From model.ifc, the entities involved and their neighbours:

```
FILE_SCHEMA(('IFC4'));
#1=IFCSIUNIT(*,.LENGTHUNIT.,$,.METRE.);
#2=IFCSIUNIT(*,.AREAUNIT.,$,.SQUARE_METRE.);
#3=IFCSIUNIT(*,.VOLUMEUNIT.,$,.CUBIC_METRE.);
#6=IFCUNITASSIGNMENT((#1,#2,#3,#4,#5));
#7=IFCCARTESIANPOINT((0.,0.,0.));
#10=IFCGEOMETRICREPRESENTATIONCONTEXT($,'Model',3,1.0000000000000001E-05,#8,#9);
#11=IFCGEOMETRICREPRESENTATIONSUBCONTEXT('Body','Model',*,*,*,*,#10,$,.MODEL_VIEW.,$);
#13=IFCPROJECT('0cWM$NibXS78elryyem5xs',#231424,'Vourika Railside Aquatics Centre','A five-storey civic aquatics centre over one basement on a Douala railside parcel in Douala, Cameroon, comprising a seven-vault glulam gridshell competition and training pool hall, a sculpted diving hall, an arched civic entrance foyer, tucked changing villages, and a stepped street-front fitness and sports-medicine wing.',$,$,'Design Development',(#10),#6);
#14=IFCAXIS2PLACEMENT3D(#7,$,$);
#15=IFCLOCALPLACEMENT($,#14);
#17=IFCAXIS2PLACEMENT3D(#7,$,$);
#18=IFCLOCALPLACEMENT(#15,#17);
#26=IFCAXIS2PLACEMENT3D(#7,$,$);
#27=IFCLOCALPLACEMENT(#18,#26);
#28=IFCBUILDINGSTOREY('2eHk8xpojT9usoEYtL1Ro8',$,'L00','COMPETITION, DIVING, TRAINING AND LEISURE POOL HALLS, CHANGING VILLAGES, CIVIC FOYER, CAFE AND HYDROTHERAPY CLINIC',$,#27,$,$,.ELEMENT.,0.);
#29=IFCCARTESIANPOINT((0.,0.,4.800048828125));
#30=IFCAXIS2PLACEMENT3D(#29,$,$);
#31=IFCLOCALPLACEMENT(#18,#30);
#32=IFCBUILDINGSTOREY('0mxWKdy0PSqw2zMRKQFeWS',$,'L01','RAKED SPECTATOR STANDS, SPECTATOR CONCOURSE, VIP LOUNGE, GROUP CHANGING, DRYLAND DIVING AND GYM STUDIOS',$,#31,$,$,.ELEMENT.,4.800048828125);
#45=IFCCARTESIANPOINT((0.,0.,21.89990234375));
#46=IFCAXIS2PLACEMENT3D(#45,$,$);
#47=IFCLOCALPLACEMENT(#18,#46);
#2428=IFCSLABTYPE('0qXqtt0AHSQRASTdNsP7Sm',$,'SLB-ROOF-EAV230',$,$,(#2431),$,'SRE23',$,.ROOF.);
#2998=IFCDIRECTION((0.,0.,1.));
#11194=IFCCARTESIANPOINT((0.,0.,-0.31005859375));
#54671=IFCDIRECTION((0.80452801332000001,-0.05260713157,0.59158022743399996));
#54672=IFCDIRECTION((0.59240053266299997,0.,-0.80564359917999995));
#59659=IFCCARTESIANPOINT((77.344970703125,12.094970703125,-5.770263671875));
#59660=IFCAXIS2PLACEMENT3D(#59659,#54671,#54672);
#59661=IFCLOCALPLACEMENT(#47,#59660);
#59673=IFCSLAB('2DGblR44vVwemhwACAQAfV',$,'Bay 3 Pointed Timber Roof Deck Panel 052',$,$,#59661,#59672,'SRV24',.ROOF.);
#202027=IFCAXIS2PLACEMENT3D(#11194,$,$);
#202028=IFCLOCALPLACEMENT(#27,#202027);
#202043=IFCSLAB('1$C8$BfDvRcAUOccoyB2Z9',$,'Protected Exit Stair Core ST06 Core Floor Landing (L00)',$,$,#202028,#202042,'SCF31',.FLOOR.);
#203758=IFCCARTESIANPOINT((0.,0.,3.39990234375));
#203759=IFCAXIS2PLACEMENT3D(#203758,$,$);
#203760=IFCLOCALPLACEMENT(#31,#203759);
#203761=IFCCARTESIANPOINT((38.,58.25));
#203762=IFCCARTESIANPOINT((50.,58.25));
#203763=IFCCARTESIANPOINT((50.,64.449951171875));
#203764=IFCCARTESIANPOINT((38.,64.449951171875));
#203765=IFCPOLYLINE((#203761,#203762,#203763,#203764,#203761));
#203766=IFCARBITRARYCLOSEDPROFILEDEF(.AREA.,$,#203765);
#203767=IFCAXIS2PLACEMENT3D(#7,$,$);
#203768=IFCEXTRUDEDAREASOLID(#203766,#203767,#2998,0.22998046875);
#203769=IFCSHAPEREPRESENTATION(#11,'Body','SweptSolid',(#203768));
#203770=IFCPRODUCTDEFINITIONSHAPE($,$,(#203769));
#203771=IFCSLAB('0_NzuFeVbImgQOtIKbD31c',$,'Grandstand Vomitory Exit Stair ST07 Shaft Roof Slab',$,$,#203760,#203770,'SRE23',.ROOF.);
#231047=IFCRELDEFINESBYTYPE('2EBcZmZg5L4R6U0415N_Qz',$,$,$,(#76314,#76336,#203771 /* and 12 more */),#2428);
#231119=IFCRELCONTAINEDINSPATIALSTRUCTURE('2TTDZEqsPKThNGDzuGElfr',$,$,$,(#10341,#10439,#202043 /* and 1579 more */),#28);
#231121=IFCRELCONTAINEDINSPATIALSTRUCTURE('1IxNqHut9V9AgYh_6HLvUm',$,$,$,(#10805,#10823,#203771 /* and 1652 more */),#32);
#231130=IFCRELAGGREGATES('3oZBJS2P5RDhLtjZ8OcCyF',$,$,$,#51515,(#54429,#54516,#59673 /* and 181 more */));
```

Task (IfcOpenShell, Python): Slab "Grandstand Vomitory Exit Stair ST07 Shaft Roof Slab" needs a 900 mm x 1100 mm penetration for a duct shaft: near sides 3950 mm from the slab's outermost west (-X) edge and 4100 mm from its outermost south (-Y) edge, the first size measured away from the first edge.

```python
import numpy as np
import ifcopenshell
import ifcopenshell.api.feature
import ifcopenshell.api.geometry
import ifcopenshell.api.root
import ifcopenshell.geom
import ifcopenshell.util.placement
import ifcopenshell.util.representation
import ifcopenshell.util.shape
import ifcopenshell.util.unit

model = ifcopenshell.open("model.ifc")
unit_scale = ifcopenshell.util.unit.calculate_unit_scale(model)
settings = ifcopenshell.geom.settings()


def volume(element):
    """Net volume in cubic metres, openings subtracted."""
    shape = ifcopenshell.geom.create_shape(settings, element)
    return ifcopenshell.util.shape.get_volume(shape.geometry)


slab = model.by_guid("0_NzuFeVbImgQOtIKbD31c")
before = volume(slab)

# Extent in the slab's own axes, in metres. The edges named are its -X and -Y sides.
slab_shape = ifcopenshell.geom.create_shape(settings, slab)
vertices = ifcopenshell.util.shape.get_vertices(slab_shape.geometry)
x_min, y_min, bottom = vertices.min(axis=0)
top = vertices[:, 2].max()

opening = ifcopenshell.api.root.create_entity(model, ifc_class="IfcOpeningElement", name="Duct shaft opening", predefined_type="OPENING")
context = ifcopenshell.util.representation.get_context(model, "Model", "Body", "MODEL_VIEW")
width, depth = 0.9, 1.1
outline = [(0.0, 0.0), (width, 0.0), (width, depth), (0.0, depth), (0.0, 0.0)]
# Overshoot both faces by 50 mm so the cut is clean.
shape = ifcopenshell.api.geometry.add_slab_representation(
    model, context=context, depth=top - bottom + 0.1, polyline=outline
)
ifcopenshell.api.geometry.assign_representation(model, product=opening, representation=shape)

matrix = ifcopenshell.util.placement.get_local_placement(slab.ObjectPlacement)
matrix[:, 3] = matrix @ np.append(np.array([x_min + 3.95, y_min + 4.1, bottom - 0.05]) / unit_scale, 1.0)
ifcopenshell.api.geometry.edit_object_placement(model, product=opening, matrix=matrix, is_si=False)
ifcopenshell.api.feature.add_feature(model, feature=opening, element=slab)

after = volume(slab)

print(f"slab volume {before:.3f} -> {after:.3f} m3")

model.write("model-out.ifc")
```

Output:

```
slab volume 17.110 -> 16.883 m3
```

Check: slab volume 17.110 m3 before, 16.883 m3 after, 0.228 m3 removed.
